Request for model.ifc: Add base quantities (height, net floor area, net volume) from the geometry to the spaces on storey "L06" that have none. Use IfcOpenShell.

First a look at what the model holds.

```python
import ifcopenshell
import ifcopenshell.util.element
import ifcopenshell.util.unit

model = ifcopenshell.open("model.ifc")
print(model.schema)
for unit_type in ("LENGTHUNIT", "AREAUNIT", "VOLUMEUNIT"):
    print(unit_type, ifcopenshell.util.unit.calculate_unit_scale(model, unit_type))
storey = next(s for s in model.by_type("IfcBuildingStorey") if s.Name == "L06")
spaces = [e for e in ifcopenshell.util.element.get_decomposition(storey) if e.is_a("IfcSpace")]
for e in sorted(spaces, key=lambda e: e.id()):
    print(e.id(), e.is_a(), e.Name, list(ifcopenshell.util.element.get_psets(e, qtos_only=True)), sep=" | ")
```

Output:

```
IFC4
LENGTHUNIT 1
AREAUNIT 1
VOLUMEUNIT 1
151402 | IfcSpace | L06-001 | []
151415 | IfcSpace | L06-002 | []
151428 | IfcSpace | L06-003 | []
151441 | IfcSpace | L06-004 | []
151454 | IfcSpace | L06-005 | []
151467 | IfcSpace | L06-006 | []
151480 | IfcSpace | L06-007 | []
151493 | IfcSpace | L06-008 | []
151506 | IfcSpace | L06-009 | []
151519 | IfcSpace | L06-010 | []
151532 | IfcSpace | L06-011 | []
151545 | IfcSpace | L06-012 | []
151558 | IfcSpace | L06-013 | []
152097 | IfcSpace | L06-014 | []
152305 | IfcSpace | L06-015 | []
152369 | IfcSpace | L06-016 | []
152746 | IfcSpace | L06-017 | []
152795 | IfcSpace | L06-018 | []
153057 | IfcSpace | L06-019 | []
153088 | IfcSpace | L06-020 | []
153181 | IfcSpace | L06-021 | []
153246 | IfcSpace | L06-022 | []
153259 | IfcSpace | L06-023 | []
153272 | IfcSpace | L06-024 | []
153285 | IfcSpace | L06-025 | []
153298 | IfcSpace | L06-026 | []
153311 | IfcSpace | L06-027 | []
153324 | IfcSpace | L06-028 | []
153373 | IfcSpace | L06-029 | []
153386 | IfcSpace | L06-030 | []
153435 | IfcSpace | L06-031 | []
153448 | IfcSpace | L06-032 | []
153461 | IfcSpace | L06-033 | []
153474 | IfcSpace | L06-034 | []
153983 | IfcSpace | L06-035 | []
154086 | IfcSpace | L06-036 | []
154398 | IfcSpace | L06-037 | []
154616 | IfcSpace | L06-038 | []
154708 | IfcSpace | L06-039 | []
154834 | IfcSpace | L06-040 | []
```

```python
import ifcopenshell
import ifcopenshell.api.pset
import ifcopenshell.geom
import ifcopenshell.util.element
import ifcopenshell.util.shape
import ifcopenshell.util.unit

model = ifcopenshell.open("model.ifc")
unit_scale = ifcopenshell.util.unit.calculate_unit_scale(model)
area_scale = ifcopenshell.util.unit.calculate_unit_scale(model, "AREAUNIT")
volume_scale = ifcopenshell.util.unit.calculate_unit_scale(model, "VOLUMEUNIT")
settings = ifcopenshell.geom.settings()

storey = next(s for s in model.by_type("IfcBuildingStorey") if s.Name == "L06")
spaces = [e for e in ifcopenshell.util.element.get_decomposition(storey) if e.is_a("IfcSpace")]

for e in sorted(spaces, key=lambda e: e.id()):
    if ifcopenshell.util.element.get_psets(e, qtos_only=True, should_inherit=False):
        continue
    # Geometry comes back in metres, in the element's own axes.
    shape = ifcopenshell.geom.create_shape(settings, e)
    values = {
        "Height": ifcopenshell.util.shape.get_z(shape.geometry) / unit_scale,
        "NetFloorArea": ifcopenshell.util.shape.get_footprint_area(shape.geometry) / area_scale,
        "NetVolume": ifcopenshell.util.shape.get_volume(shape.geometry) / volume_scale,
    }
    qto = ifcopenshell.api.pset.add_qto(model, product=e, name="Qto_SpaceBaseQuantities")
    ifcopenshell.api.pset.edit_qto(model, qto=qto, properties=values)
    print(e.id(), {k: round(v, 3) for k, v in values.items()})

model.write("model_v2.ifc")
```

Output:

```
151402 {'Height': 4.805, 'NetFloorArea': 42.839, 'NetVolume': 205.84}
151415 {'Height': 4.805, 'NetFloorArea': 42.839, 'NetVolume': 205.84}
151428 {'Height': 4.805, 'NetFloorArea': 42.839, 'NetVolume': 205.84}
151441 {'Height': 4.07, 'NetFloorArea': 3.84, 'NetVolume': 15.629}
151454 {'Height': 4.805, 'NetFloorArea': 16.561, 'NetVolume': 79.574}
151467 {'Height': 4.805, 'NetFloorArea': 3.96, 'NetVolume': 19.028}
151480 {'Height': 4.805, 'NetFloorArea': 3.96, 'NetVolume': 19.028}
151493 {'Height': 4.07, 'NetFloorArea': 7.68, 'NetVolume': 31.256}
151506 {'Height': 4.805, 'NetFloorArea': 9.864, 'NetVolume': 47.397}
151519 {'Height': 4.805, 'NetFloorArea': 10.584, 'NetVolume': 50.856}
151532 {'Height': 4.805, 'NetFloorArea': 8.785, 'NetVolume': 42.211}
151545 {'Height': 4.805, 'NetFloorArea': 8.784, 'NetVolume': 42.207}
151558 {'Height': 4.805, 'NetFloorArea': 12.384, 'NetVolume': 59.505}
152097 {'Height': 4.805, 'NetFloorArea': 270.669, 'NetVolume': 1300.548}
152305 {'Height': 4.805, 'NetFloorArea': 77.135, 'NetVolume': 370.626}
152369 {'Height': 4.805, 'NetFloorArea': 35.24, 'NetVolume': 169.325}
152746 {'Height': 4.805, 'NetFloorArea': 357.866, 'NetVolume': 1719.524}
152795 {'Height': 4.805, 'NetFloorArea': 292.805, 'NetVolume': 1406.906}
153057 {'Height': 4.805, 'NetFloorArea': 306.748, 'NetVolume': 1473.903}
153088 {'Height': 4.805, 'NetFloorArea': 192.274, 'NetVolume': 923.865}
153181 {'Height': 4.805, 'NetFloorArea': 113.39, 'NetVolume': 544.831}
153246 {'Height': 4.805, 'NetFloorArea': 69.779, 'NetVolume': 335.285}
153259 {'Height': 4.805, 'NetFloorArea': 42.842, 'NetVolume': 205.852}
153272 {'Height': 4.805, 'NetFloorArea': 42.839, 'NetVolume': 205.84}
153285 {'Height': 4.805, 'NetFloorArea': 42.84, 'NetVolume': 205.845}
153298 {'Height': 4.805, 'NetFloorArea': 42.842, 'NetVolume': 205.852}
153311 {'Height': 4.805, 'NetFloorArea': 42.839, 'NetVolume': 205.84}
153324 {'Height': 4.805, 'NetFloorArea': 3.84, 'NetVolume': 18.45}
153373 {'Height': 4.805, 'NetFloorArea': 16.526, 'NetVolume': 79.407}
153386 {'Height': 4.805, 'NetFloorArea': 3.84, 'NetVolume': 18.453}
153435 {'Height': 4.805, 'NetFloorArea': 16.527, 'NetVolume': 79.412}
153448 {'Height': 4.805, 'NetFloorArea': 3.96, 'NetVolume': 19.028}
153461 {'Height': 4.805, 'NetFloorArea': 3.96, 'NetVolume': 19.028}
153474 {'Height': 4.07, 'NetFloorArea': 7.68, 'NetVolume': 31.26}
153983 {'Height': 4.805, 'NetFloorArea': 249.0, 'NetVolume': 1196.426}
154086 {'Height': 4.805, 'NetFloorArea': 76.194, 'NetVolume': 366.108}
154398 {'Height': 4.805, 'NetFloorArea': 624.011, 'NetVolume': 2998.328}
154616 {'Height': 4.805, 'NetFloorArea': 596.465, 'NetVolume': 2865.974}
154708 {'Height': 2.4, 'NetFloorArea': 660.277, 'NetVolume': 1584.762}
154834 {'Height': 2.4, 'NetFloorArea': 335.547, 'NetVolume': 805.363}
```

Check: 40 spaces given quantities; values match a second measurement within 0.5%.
